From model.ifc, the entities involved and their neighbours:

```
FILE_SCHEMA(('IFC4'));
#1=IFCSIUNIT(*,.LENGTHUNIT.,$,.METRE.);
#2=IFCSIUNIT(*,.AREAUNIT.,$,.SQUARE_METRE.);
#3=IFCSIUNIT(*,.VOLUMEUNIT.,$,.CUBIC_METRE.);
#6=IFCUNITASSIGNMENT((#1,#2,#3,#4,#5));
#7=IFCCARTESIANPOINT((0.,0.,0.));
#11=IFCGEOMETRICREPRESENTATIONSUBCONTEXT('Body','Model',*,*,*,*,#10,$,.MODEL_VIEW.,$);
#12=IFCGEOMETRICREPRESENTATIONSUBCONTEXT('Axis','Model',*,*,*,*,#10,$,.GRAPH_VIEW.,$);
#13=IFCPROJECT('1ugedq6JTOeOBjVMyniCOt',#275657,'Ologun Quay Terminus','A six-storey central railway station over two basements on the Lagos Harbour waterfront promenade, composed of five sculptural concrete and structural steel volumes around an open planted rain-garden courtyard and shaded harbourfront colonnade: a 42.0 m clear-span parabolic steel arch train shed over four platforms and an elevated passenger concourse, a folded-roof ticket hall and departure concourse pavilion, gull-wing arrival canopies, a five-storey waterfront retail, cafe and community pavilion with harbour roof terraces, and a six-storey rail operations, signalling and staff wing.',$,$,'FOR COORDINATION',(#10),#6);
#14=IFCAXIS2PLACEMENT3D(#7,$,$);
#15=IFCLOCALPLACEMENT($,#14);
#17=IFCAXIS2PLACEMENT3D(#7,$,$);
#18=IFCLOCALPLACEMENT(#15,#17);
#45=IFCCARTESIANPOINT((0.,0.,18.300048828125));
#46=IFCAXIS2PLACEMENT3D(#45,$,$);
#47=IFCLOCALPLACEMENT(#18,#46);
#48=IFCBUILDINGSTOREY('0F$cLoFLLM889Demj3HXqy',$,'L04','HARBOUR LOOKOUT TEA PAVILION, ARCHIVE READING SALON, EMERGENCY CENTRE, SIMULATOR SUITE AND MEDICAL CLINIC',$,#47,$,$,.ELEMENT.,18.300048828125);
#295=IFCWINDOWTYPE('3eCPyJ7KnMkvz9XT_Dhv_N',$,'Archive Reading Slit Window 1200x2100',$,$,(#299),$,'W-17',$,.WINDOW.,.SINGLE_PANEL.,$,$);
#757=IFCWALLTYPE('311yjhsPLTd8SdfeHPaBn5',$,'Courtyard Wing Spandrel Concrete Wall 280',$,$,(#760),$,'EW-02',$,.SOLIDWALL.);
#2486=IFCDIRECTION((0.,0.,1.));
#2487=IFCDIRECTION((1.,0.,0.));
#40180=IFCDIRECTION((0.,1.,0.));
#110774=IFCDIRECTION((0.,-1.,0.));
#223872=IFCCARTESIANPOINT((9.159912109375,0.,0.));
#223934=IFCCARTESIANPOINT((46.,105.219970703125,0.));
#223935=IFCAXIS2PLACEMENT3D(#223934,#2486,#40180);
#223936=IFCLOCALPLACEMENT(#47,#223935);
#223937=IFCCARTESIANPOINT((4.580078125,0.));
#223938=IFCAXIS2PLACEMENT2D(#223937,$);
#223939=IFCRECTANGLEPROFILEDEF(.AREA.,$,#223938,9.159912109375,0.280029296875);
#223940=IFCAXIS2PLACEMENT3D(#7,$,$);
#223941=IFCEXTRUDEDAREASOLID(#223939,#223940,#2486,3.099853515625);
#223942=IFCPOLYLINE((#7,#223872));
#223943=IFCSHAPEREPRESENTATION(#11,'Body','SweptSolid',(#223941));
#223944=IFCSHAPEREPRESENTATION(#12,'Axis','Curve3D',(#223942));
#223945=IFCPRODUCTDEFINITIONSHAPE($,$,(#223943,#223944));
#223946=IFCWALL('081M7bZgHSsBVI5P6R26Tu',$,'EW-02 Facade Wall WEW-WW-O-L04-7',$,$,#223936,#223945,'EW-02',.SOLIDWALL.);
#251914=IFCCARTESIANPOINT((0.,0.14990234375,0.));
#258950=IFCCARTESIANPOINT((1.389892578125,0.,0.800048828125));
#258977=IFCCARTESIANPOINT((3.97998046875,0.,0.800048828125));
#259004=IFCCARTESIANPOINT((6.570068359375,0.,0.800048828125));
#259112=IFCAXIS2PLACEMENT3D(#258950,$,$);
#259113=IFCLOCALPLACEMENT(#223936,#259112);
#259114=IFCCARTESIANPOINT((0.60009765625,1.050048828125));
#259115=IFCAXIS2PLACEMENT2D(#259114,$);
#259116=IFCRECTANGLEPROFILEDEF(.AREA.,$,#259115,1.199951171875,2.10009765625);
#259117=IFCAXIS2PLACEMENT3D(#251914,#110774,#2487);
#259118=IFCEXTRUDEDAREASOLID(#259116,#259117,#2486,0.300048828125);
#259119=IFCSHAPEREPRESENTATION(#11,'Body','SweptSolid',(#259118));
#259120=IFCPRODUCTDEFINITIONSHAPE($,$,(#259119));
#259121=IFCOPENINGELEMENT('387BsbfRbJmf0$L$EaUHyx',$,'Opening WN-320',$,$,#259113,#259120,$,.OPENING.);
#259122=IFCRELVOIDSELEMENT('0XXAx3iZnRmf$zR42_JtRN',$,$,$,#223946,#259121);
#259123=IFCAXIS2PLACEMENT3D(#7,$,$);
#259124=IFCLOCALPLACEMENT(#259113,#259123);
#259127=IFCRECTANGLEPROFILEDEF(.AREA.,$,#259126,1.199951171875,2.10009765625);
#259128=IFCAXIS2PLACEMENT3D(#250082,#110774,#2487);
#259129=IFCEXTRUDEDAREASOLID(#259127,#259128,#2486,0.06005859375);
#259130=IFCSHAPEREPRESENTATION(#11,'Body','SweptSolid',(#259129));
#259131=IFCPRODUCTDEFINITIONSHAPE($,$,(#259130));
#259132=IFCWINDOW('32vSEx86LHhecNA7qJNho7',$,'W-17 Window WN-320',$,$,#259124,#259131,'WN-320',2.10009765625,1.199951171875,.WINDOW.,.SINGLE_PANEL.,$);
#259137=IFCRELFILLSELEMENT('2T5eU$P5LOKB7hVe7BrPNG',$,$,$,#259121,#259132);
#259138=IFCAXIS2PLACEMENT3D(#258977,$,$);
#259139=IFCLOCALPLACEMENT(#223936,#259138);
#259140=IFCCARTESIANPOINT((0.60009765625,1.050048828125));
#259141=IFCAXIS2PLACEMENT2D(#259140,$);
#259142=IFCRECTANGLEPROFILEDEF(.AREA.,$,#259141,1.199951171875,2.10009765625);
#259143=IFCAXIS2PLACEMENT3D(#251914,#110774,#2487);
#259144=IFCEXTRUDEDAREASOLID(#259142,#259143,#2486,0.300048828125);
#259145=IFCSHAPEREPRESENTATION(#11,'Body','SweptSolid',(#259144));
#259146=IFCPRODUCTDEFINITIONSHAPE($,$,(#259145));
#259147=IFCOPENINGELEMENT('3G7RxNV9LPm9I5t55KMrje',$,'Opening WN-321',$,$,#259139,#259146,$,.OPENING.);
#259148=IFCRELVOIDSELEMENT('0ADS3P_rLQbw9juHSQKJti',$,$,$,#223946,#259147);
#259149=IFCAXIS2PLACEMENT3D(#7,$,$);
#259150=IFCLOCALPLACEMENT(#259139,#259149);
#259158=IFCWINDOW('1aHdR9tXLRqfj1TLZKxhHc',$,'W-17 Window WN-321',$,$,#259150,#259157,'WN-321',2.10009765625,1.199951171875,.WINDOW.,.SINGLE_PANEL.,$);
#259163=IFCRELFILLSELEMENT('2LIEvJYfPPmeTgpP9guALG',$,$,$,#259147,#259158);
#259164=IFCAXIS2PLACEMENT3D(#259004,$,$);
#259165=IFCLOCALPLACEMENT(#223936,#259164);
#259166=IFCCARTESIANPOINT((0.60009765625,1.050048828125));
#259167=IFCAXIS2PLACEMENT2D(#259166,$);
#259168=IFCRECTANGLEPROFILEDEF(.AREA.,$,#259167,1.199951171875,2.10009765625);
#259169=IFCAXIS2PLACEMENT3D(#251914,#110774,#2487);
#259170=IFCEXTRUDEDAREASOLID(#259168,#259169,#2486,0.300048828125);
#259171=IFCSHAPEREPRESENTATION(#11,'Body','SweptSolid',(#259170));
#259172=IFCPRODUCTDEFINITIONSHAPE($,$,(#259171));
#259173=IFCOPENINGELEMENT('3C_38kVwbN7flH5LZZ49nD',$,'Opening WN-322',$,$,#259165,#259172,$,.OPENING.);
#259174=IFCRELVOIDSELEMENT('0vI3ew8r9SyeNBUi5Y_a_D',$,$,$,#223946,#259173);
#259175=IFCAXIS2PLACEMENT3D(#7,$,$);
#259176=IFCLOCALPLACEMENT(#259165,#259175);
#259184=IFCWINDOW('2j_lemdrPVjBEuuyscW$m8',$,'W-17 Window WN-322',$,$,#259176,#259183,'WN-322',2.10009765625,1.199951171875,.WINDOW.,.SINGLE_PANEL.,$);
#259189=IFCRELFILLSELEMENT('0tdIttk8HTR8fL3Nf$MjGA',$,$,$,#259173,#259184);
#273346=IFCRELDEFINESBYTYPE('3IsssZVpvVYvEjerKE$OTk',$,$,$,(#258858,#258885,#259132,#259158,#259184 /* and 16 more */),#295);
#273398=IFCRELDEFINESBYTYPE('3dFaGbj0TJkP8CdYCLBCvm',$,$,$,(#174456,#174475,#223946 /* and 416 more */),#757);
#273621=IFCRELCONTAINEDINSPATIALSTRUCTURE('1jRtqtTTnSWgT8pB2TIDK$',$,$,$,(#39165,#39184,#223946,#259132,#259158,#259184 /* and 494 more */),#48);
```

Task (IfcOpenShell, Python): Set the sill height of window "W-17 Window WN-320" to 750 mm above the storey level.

```python
import numpy as np
import ifcopenshell
import ifcopenshell.api.geometry
import ifcopenshell.geom
import ifcopenshell.util.element
import ifcopenshell.util.placement
import ifcopenshell.util.shape
import ifcopenshell.util.unit

model = ifcopenshell.open("model.ifc")
unit_scale = ifcopenshell.util.unit.calculate_unit_scale(model)

window = model.by_guid("32vSEx86LHhecNA7qJNho7")
opening = window.FillsVoids[0].RelatingOpeningElement
storey = ifcopenshell.util.element.get_container(window, ifc_class="IfcBuildingStorey")
level = ifcopenshell.util.placement.get_local_placement(storey.ObjectPlacement)[2, 3]

# The opening's origin need not be at the sill, so measure its lowest point.
shape = ifcopenshell.geom.create_shape(ifcopenshell.geom.settings(), opening)
bottom = ifcopenshell.util.shape.get_shape_bottom_elevation(shape, shape.geometry) / unit_scale
dz = level + 0.75 / unit_scale - bottom

shift = np.array([0.0, 0.0, dz])
# The window is placed relative to its opening, so it follows when the opening moves.
matrix = ifcopenshell.util.placement.get_local_placement(opening.ObjectPlacement)
matrix[:3, 3] += shift
ifcopenshell.api.geometry.edit_object_placement(
    model, product=opening, matrix=matrix, is_si=False, should_transform_children=True
)

print(f"moved by {dz * unit_scale:+.3f} m")

model.write("model_updated.ifc")
```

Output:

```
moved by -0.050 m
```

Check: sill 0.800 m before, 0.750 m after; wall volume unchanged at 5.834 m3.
